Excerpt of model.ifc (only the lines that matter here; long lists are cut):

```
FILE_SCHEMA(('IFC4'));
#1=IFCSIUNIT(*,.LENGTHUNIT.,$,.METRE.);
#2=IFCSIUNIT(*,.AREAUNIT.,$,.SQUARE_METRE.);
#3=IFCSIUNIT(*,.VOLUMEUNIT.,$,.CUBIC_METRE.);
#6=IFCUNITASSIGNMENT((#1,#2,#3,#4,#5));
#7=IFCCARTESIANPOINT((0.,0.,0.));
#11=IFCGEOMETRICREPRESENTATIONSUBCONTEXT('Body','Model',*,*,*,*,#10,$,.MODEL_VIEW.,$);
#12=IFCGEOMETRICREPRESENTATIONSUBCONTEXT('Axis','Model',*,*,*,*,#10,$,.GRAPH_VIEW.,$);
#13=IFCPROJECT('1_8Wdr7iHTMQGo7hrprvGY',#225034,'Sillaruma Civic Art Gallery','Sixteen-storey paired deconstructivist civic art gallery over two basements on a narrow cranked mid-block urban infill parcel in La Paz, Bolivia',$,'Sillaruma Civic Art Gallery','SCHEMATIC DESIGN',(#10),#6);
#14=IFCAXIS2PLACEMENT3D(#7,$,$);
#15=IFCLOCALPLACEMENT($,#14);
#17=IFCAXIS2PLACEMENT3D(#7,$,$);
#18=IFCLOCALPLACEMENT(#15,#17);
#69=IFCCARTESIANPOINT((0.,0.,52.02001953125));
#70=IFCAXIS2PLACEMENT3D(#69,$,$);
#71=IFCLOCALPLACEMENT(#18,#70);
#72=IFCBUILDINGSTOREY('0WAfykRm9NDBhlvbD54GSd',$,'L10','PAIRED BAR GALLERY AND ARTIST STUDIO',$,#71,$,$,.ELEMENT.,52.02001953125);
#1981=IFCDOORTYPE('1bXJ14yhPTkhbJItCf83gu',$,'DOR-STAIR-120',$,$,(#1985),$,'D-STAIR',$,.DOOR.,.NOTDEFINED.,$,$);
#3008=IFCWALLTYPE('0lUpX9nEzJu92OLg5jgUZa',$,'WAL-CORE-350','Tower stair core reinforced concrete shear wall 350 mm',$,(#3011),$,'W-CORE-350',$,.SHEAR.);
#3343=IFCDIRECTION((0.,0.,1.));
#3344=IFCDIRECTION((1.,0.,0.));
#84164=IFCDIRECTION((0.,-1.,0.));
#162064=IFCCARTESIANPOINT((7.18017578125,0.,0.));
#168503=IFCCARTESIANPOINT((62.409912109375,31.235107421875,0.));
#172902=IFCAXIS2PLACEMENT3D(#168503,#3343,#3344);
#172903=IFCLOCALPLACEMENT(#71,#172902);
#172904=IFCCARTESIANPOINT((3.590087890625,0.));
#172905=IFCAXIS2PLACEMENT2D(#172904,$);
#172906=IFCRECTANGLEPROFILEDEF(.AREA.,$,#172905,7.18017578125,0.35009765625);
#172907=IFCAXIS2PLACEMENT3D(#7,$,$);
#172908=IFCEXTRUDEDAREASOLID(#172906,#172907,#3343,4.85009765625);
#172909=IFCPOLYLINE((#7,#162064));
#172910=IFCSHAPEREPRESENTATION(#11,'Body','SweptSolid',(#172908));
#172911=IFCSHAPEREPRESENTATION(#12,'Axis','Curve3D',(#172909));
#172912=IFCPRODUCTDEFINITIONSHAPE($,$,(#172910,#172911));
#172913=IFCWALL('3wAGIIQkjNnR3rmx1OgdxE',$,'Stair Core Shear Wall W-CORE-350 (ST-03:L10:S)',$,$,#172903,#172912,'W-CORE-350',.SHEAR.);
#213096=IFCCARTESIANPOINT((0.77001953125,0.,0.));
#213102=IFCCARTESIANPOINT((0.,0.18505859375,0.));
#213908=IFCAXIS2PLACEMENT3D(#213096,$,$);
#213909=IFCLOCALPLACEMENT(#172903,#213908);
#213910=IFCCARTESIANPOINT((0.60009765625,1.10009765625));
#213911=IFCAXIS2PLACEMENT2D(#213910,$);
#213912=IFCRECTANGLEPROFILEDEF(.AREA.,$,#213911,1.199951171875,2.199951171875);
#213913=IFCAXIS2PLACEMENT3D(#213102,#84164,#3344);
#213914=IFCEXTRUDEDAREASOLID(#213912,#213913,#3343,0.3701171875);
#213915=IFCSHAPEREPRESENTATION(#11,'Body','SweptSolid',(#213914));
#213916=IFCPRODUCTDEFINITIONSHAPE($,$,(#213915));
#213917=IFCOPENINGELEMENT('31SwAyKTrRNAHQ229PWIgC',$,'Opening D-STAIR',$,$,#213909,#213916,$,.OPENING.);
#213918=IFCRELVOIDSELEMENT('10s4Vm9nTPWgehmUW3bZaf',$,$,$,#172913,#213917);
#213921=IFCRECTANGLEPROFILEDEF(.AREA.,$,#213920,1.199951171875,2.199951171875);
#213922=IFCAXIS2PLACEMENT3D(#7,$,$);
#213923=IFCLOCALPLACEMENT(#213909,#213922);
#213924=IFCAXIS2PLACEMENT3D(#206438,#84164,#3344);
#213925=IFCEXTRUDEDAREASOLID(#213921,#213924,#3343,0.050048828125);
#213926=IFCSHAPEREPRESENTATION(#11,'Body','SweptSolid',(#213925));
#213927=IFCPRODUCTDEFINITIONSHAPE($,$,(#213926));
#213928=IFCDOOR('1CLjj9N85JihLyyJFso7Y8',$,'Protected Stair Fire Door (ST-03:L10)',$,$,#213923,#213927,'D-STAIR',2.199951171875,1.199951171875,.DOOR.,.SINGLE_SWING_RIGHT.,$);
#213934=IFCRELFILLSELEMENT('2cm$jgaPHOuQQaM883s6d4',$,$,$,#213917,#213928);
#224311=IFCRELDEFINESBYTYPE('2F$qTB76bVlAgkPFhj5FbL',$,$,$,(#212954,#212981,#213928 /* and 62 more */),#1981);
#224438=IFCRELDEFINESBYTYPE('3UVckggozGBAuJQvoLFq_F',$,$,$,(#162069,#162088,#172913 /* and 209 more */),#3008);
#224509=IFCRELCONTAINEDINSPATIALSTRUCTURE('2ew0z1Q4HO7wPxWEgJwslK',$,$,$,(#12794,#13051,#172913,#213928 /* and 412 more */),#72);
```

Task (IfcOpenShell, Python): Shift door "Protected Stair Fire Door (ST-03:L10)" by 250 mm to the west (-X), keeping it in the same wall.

```python
import ifcopenshell
import ifcopenshell.api.geometry
import ifcopenshell.util.placement
import ifcopenshell.util.unit

model = ifcopenshell.open("model.ifc")
unit_scale = ifcopenshell.util.unit.calculate_unit_scale(model)

door = model.by_guid("1CLjj9N85JihLyyJFso7Y8")
opening = door.FillsVoids[0].RelatingOpeningElement
wall = opening.VoidsElements[0].RelatingBuildingElement

wall_matrix = ifcopenshell.util.placement.get_local_placement(wall.ObjectPlacement)
shift = wall_matrix[:3, 0] * -0.25 / unit_scale
before = ifcopenshell.util.placement.get_local_placement(door.ObjectPlacement)[:3, 3].copy()

# The door is placed relative to its opening, so it follows when the opening moves.
matrix = ifcopenshell.util.placement.get_local_placement(opening.ObjectPlacement)
matrix[:3, 3] += shift
ifcopenshell.api.geometry.edit_object_placement(
    model, product=opening, matrix=matrix, is_si=False, should_transform_children=True
)

after = ifcopenshell.util.placement.get_local_placement(door.ObjectPlacement)[:3, 3]
print("door moved by", (after - before).round(3) + 0.0)

model.write("model_updated.ifc")
```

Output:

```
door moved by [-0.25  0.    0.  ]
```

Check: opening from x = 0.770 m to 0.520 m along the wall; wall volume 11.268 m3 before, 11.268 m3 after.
